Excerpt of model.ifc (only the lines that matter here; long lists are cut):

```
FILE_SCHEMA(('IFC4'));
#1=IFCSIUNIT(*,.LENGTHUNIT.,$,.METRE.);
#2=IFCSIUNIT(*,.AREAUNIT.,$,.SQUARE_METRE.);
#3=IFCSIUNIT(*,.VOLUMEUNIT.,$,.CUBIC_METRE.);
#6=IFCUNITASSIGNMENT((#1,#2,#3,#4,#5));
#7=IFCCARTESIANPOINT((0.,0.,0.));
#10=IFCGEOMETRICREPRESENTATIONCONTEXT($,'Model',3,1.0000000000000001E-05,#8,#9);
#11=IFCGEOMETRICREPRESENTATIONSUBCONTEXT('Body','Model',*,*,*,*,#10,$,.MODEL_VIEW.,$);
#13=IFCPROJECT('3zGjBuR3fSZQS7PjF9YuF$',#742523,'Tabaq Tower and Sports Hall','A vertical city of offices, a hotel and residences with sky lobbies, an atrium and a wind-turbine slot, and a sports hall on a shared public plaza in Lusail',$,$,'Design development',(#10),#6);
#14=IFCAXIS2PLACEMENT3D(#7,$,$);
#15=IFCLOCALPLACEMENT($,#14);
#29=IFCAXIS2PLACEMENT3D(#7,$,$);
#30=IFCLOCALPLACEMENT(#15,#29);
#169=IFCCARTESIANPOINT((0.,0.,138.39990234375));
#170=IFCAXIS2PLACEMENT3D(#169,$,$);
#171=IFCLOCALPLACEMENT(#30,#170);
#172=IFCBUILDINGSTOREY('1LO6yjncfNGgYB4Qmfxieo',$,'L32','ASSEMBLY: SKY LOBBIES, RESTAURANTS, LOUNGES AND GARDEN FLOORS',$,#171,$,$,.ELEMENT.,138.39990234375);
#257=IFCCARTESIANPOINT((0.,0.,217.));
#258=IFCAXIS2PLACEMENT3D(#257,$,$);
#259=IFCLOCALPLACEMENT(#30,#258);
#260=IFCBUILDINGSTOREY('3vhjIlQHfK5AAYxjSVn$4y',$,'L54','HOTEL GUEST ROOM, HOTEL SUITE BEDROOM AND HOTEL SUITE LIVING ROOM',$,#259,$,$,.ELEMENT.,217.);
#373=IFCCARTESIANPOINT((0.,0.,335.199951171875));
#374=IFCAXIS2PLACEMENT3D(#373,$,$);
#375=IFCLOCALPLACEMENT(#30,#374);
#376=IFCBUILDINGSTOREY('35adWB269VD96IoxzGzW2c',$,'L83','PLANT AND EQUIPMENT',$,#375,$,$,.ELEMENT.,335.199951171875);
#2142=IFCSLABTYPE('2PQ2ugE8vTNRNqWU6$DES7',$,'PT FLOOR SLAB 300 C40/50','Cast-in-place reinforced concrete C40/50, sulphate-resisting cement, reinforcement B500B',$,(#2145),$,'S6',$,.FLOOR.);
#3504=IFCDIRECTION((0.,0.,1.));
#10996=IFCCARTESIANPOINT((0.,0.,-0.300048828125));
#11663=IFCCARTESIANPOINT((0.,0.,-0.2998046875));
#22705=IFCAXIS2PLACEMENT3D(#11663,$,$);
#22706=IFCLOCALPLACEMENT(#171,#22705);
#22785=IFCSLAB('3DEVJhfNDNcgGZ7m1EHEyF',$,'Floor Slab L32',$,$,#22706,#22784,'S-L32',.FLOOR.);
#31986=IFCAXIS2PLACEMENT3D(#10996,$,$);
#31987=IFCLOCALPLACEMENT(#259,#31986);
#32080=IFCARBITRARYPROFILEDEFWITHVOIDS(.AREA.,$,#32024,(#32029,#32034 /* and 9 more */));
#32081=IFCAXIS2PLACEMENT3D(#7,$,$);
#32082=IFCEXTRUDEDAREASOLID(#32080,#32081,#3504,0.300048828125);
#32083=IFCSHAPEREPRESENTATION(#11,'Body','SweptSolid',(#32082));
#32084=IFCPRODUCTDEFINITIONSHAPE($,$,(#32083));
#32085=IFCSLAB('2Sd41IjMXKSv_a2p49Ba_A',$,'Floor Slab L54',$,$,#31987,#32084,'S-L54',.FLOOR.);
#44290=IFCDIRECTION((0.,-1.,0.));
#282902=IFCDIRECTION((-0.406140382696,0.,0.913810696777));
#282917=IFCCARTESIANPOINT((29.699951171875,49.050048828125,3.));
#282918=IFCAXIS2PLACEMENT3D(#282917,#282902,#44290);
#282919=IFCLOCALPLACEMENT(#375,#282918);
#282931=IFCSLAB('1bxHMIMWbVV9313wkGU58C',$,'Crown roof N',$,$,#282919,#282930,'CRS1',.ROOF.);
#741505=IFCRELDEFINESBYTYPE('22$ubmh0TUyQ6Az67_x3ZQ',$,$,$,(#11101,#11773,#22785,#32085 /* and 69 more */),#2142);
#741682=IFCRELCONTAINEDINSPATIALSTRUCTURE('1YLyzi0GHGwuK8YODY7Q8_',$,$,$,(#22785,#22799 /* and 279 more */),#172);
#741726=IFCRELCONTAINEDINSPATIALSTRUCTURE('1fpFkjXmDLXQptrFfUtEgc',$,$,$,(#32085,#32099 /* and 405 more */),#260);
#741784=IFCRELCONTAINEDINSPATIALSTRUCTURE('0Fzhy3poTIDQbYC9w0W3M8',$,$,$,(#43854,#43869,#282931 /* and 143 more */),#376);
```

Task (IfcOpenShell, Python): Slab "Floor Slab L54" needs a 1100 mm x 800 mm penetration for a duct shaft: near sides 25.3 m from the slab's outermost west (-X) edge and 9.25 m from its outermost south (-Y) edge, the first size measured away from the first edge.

```python
import numpy as np
import ifcopenshell
import ifcopenshell.api.feature
import ifcopenshell.api.geometry
import ifcopenshell.api.root
import ifcopenshell.geom
import ifcopenshell.util.placement
import ifcopenshell.util.representation
import ifcopenshell.util.shape
import ifcopenshell.util.unit

model = ifcopenshell.open("model.ifc")
unit_scale = ifcopenshell.util.unit.calculate_unit_scale(model)
settings = ifcopenshell.geom.settings()


def volume(element):
    """Net volume in cubic metres, openings subtracted."""
    shape = ifcopenshell.geom.create_shape(settings, element)
    return ifcopenshell.util.shape.get_volume(shape.geometry)


slab = model.by_id(32085)
before = volume(slab)

# Extent in the slab's own axes, in metres. The edges named are its -X and -Y sides.
slab_shape = ifcopenshell.geom.create_shape(settings, slab)
vertices = ifcopenshell.util.shape.get_vertices(slab_shape.geometry)
x_min, y_min, bottom = vertices.min(axis=0)
top = vertices[:, 2].max()

opening = ifcopenshell.api.root.create_entity(model, ifc_class="IfcOpeningElement", name="Duct shaft opening", predefined_type="OPENING")
context = ifcopenshell.util.representation.get_context(model, "Model", "Body", "MODEL_VIEW")
width, depth = 1.1, 0.8
outline = [(0.0, 0.0), (width, 0.0), (width, depth), (0.0, depth), (0.0, 0.0)]
# Overshoot both faces by 50 mm so the cut is clean.
shape = ifcopenshell.api.geometry.add_slab_representation(
    model, context=context, depth=top - bottom + 0.1, polyline=outline
)
ifcopenshell.api.geometry.assign_representation(model, product=opening, representation=shape)

matrix = ifcopenshell.util.placement.get_local_placement(slab.ObjectPlacement)
matrix[:, 3] = matrix @ np.append(np.array([x_min + 25.3, y_min + 9.25, bottom - 0.05]) / unit_scale, 1.0)
ifcopenshell.api.geometry.edit_object_placement(model, product=opening, matrix=matrix, is_si=False)
ifcopenshell.api.feature.add_feature(model, feature=opening, element=slab)

after = volume(slab)

print(f"slab volume {before:.3f} -> {after:.3f} m3")

model.write("model_updated.ifc")
```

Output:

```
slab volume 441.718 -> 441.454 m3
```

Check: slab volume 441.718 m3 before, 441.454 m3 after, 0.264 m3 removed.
